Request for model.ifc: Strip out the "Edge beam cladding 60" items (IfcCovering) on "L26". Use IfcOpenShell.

First a look at what the model holds.

```python
import ifcopenshell
import ifcopenshell.util.element

model = ifcopenshell.open("model.ifc")
print(model.schema)
storey = next(s for s in model.by_type("IfcBuildingStorey") if s.Name == "L26")
coverings = [e for e in ifcopenshell.util.element.get_decomposition(storey) if e.is_a("IfcCovering")]
seen = {}
for e in coverings:
    element_type = ifcopenshell.util.element.get_type(e)
    name = element_type.Name if element_type not in (None, e) else None
    seen[name] = seen.get(name, 0) + 1
for name, count in sorted(seen.items(), key=str):
    print(count, "x", name)
```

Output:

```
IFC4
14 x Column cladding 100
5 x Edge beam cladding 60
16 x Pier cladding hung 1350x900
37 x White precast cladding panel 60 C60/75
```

```python
import ifcopenshell
import ifcopenshell.api.root
import ifcopenshell.util.element

model = ifcopenshell.open("model.ifc")

storey = next(s for s in model.by_type("IfcBuildingStorey") if s.Name == "L26")
coverings = [e for e in ifcopenshell.util.element.get_decomposition(storey) if e.is_a("IfcCovering")]
targets = [e for e in coverings if (t := ifcopenshell.util.element.get_type(e)) not in (None, e) and t.Name == "Edge beam cladding 60"]

for e in targets:
    ifcopenshell.api.root.remove_product(model, product=e)
print(len(targets), "removed")

model.write("model_rev.ifc")
```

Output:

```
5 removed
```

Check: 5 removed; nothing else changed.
